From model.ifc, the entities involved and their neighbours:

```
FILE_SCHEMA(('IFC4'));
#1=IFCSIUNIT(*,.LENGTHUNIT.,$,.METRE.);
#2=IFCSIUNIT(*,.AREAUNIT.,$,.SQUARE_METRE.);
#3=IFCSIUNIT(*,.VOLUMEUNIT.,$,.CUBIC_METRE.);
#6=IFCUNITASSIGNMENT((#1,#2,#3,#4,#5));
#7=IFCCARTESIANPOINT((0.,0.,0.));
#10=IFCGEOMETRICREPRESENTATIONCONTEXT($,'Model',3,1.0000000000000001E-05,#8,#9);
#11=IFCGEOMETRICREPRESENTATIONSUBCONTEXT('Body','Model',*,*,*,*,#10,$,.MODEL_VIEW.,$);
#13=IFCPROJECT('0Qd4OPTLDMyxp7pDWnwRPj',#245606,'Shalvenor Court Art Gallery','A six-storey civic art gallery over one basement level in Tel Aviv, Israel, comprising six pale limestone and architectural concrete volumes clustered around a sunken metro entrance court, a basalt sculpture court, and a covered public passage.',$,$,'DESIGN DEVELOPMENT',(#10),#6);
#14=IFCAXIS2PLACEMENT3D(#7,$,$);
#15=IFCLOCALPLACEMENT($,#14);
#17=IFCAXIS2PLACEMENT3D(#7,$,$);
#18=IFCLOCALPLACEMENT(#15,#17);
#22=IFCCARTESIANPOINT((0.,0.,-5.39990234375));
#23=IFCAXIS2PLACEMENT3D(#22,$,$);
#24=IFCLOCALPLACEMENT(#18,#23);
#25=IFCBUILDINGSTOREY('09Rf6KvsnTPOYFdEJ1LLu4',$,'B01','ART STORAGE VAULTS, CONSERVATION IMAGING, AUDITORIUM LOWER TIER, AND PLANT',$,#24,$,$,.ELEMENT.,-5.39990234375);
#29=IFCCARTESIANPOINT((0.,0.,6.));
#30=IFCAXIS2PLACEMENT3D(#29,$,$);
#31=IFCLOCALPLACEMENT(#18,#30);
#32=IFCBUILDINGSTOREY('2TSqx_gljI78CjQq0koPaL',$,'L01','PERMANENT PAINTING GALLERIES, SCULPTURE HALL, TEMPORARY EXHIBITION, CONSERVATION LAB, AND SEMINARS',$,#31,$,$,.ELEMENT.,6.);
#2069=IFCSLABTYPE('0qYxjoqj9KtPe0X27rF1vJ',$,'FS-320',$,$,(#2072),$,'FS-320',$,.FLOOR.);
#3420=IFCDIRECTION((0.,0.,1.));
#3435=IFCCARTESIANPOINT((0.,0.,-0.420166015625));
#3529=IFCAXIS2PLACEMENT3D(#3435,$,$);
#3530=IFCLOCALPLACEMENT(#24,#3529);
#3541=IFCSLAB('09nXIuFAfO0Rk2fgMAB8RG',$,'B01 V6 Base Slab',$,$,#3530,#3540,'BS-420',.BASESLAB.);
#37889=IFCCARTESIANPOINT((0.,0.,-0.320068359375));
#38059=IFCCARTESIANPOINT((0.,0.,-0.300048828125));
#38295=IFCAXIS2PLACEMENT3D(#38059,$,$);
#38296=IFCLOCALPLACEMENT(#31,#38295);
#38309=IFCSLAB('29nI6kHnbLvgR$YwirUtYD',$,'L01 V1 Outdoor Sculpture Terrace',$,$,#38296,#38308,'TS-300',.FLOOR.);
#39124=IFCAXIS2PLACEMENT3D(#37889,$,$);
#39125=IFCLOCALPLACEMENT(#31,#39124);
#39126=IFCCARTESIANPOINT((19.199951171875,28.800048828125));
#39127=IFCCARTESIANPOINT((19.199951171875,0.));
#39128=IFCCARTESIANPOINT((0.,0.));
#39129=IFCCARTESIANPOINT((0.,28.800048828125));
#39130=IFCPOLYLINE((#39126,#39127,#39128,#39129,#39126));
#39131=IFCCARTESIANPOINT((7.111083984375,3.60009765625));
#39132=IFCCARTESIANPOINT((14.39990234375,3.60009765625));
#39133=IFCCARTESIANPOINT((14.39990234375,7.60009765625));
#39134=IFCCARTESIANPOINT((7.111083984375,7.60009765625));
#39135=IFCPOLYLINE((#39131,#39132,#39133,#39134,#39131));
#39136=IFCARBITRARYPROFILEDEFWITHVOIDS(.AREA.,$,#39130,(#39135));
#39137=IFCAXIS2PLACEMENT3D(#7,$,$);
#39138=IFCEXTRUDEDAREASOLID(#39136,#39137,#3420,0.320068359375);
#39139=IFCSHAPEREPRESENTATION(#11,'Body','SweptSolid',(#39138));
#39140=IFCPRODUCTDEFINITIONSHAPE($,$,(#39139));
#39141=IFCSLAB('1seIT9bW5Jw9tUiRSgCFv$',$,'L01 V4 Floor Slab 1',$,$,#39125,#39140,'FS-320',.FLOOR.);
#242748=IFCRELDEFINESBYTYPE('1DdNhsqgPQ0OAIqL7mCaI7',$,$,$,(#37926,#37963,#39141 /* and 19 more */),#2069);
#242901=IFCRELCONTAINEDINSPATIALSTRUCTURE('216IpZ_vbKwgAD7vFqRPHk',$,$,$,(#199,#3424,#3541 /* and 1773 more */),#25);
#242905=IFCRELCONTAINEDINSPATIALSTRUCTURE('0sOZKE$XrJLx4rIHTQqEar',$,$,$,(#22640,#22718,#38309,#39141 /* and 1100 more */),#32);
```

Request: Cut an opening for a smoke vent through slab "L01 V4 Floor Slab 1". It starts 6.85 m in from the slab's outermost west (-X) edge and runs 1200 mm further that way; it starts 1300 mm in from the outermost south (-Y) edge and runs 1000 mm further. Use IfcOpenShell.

```python
import numpy as np
import ifcopenshell
import ifcopenshell.api.feature
import ifcopenshell.api.geometry
import ifcopenshell.api.root
import ifcopenshell.geom
import ifcopenshell.util.placement
import ifcopenshell.util.representation
import ifcopenshell.util.shape
import ifcopenshell.util.unit

model = ifcopenshell.open("model.ifc")
unit_scale = ifcopenshell.util.unit.calculate_unit_scale(model)
settings = ifcopenshell.geom.settings()


def volume(element):
    """Net volume in cubic metres, openings subtracted."""
    shape = ifcopenshell.geom.create_shape(settings, element)
    return ifcopenshell.util.shape.get_volume(shape.geometry)


slab = model.by_guid("1seIT9bW5Jw9tUiRSgCFv$")
before = volume(slab)

# Extent in the slab's own axes, in metres. The edges named are its -X and -Y sides.
slab_shape = ifcopenshell.geom.create_shape(settings, slab)
vertices = ifcopenshell.util.shape.get_vertices(slab_shape.geometry)
x_min, y_min, bottom = vertices.min(axis=0)
top = vertices[:, 2].max()

opening = ifcopenshell.api.root.create_entity(model, ifc_class="IfcOpeningElement", name="Smoke vent opening", predefined_type="OPENING")
context = ifcopenshell.util.representation.get_context(model, "Model", "Body", "MODEL_VIEW")
width, depth = 1.2, 1
outline = [(0.0, 0.0), (width, 0.0), (width, depth), (0.0, depth), (0.0, 0.0)]
# Overshoot both faces by 50 mm so the cut is clean.
shape = ifcopenshell.api.geometry.add_slab_representation(
    model, context=context, depth=top - bottom + 0.1, polyline=outline
)
ifcopenshell.api.geometry.assign_representation(model, product=opening, representation=shape)

matrix = ifcopenshell.util.placement.get_local_placement(slab.ObjectPlacement)
matrix[:, 3] = matrix @ np.append(np.array([x_min + 6.85, y_min + 1.3, bottom - 0.05]) / unit_scale, 1.0)
ifcopenshell.api.geometry.edit_object_placement(model, product=opening, matrix=matrix, is_si=False)
ifcopenshell.api.feature.add_feature(model, feature=opening, element=slab)

after = volume(slab)

print(f"slab volume {before:.3f} -> {after:.3f} m3")

model.write("model_updated.ifc")
```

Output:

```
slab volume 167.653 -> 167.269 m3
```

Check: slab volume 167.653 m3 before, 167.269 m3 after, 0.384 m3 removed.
